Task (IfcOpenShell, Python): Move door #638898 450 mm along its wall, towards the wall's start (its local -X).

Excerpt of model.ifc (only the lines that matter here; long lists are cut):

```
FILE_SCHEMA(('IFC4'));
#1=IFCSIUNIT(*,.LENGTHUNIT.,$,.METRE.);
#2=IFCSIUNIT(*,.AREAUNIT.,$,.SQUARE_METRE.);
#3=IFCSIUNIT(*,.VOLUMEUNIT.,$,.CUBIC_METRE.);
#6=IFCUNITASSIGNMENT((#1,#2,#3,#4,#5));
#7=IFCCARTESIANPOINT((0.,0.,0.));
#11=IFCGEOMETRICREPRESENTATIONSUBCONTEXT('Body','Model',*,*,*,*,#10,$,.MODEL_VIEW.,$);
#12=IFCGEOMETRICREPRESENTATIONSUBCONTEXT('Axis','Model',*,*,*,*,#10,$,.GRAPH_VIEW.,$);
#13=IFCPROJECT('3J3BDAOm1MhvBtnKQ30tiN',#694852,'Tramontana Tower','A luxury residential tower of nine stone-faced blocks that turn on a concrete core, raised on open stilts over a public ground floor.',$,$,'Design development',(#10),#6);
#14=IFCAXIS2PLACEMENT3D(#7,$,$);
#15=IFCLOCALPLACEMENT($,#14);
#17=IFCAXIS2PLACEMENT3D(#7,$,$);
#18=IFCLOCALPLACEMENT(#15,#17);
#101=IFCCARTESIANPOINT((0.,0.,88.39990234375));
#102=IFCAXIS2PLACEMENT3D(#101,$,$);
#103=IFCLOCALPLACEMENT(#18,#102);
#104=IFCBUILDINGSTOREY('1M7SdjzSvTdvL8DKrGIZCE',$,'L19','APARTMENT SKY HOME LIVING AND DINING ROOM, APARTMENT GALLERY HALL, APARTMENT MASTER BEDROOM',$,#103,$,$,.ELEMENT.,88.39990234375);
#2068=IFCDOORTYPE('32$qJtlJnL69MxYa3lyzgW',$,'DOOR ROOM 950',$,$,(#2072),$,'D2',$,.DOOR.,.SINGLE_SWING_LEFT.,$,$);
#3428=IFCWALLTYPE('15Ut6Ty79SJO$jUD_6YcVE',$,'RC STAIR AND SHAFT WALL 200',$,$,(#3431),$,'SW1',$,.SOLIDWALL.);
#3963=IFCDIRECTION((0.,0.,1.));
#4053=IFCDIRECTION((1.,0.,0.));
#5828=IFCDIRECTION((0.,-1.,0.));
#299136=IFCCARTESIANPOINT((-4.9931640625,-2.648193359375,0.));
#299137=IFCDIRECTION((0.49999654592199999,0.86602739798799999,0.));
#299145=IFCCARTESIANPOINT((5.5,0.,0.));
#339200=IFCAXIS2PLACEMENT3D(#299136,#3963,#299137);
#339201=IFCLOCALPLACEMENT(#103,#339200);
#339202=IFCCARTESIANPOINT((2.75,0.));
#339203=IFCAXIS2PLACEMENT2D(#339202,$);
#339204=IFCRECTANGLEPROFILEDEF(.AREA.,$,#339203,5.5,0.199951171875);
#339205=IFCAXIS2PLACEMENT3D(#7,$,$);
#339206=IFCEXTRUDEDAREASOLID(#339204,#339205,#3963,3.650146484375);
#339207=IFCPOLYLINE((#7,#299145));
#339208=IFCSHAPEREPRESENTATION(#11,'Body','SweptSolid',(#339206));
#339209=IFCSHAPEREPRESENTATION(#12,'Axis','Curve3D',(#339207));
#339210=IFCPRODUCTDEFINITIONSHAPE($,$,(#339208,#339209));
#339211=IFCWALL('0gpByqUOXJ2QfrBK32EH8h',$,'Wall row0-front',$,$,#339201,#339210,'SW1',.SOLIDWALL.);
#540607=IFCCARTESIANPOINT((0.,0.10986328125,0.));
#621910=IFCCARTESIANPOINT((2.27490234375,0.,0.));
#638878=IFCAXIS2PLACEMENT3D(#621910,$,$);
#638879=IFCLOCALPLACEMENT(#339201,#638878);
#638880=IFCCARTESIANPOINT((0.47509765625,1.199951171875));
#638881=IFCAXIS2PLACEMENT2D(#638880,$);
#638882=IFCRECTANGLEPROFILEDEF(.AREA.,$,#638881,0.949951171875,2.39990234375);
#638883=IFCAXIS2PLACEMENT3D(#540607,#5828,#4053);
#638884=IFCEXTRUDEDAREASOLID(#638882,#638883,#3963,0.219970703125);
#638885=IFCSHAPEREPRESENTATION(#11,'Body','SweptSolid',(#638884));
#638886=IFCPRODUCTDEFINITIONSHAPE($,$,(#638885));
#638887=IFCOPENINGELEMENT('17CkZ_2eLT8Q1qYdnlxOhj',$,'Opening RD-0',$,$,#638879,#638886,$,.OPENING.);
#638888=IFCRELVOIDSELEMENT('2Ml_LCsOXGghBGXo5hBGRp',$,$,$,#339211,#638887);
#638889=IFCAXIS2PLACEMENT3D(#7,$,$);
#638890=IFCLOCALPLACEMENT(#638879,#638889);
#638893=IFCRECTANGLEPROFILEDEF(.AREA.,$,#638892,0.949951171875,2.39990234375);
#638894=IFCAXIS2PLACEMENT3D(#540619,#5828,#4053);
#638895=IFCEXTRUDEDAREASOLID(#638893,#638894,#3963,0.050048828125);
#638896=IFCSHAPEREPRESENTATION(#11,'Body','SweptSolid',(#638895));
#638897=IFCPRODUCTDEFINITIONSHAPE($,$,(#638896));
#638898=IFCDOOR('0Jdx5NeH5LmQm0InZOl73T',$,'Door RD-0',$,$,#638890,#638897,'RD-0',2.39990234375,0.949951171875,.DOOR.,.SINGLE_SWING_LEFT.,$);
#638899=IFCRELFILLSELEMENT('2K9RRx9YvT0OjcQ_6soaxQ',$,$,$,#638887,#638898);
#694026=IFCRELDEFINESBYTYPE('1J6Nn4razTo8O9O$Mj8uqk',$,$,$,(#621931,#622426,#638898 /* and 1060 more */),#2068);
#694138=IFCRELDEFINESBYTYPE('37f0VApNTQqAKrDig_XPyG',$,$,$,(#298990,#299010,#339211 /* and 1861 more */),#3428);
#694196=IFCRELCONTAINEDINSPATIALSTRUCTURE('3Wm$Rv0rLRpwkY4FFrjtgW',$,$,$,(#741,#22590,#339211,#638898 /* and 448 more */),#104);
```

```python
import ifcopenshell
import ifcopenshell.api.geometry
import ifcopenshell.util.placement
import ifcopenshell.util.unit

model = ifcopenshell.open("model.ifc")
unit_scale = ifcopenshell.util.unit.calculate_unit_scale(model)

door = model.by_guid("0Jdx5NeH5LmQm0InZOl73T")
opening = door.FillsVoids[0].RelatingOpeningElement
wall = opening.VoidsElements[0].RelatingBuildingElement

wall_matrix = ifcopenshell.util.placement.get_local_placement(wall.ObjectPlacement)
shift = wall_matrix[:3, 0] * -0.45 / unit_scale
before = ifcopenshell.util.placement.get_local_placement(door.ObjectPlacement)[:3, 3].copy()

# The door is placed relative to its opening, so it follows when the opening moves.
matrix = ifcopenshell.util.placement.get_local_placement(opening.ObjectPlacement)
matrix[:3, 3] += shift
ifcopenshell.api.geometry.edit_object_placement(
    model, product=opening, matrix=matrix, is_si=False, should_transform_children=True
)

after = ifcopenshell.util.placement.get_local_placement(door.ObjectPlacement)[:3, 3]
print("door moved by", (after - before).round(3) + 0.0)

model.write("model_v2.ifc")
```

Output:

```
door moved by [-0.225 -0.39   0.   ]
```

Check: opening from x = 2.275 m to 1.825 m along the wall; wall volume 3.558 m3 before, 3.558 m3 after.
